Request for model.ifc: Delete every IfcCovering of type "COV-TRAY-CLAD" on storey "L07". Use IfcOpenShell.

First a look at what the model holds.

```python
import ifcopenshell
import ifcopenshell.util.element

model = ifcopenshell.open("model.ifc")
print(model.schema)
storey = next(s for s in model.by_type("IfcBuildingStorey") if s.Name == "L07")
coverings = [e for e in ifcopenshell.util.element.get_decomposition(storey) if e.is_a("IfcCovering")]
seen = {}
for e in coverings:
    element_type = ifcopenshell.util.element.get_type(e)
    name = element_type.Name if element_type not in (None, e) else None
    seen[name] = seen.get(name, 0) + 1
for name, count in sorted(seen.items(), key=str):
    print(count, "x", name)
```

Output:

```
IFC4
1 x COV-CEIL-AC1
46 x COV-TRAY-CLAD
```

```python
import ifcopenshell
import ifcopenshell.api.root
import ifcopenshell.util.element

model = ifcopenshell.open("model.ifc")

storey = next(s for s in model.by_type("IfcBuildingStorey") if s.Name == "L07")
coverings = [e for e in ifcopenshell.util.element.get_decomposition(storey) if e.is_a("IfcCovering")]
targets = [e for e in coverings if (t := ifcopenshell.util.element.get_type(e)) not in (None, e) and t.Name == "COV-TRAY-CLAD"]

for e in targets:
    ifcopenshell.api.root.remove_product(model, product=e)
print(len(targets), "removed")

model.write("model_edited.ifc")
```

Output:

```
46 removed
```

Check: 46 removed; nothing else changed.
